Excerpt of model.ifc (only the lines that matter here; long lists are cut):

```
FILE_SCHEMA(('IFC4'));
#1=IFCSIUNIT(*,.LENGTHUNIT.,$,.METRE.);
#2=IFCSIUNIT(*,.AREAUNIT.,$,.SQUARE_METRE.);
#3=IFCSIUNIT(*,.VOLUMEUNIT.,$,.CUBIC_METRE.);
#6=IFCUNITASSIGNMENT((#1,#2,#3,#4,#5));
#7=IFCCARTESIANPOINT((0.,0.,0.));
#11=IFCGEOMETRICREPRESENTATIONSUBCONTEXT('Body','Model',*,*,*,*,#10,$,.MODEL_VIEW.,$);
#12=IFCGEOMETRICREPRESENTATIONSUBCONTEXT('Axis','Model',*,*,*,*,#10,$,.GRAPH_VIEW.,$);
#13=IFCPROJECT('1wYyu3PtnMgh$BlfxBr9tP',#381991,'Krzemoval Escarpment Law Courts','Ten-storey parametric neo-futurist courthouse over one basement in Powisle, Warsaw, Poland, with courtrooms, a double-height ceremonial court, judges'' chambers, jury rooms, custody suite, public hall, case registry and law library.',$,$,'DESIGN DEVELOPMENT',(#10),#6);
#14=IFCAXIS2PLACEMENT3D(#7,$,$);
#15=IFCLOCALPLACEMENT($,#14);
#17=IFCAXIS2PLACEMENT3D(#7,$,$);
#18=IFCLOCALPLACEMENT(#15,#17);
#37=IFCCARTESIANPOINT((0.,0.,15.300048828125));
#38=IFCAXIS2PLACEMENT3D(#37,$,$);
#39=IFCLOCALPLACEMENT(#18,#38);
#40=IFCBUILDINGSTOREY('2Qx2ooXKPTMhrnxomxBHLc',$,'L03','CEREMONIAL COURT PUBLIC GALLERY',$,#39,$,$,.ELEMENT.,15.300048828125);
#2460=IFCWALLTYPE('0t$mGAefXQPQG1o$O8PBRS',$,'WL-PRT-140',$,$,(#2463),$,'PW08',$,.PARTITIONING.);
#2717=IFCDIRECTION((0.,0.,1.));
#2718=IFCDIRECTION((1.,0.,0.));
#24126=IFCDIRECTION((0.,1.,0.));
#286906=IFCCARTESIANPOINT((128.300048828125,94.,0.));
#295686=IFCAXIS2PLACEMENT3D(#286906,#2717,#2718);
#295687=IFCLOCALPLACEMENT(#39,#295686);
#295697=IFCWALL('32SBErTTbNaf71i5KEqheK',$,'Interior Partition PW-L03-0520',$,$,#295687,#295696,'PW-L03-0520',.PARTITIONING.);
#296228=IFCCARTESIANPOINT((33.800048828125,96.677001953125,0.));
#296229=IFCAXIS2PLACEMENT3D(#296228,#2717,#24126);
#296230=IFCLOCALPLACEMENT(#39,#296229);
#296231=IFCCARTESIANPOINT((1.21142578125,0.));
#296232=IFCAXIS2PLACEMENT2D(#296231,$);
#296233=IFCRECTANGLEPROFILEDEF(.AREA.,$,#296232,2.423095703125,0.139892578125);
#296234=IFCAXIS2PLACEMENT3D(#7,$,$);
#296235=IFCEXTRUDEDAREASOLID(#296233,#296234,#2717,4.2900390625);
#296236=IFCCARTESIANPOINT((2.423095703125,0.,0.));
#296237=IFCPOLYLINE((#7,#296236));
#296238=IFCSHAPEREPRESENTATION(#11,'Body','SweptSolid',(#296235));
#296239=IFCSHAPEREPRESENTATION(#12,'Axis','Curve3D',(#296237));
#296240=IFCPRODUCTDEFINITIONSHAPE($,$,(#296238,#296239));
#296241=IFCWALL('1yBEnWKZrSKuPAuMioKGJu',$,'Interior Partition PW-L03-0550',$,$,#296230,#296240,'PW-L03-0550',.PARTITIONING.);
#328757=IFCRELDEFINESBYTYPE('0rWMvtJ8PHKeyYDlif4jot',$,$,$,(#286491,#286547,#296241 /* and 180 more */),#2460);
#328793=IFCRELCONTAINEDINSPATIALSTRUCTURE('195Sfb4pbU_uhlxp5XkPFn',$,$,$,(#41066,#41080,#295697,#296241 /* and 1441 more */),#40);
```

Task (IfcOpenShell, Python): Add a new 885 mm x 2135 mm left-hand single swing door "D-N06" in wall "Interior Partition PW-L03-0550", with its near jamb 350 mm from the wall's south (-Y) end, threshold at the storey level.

```python
import numpy as np
import ifcopenshell
import ifcopenshell.api.feature
import ifcopenshell.api.geometry
import ifcopenshell.api.root
import ifcopenshell.api.spatial
import ifcopenshell.geom
import ifcopenshell.util.element
import ifcopenshell.util.placement
import ifcopenshell.util.representation
import ifcopenshell.util.shape
import ifcopenshell.util.unit

model = ifcopenshell.open("model.ifc")
unit_scale = ifcopenshell.util.unit.calculate_unit_scale(model)
settings = ifcopenshell.geom.settings()


def volume(element):
    """Net volume in cubic metres, openings subtracted."""
    shape = ifcopenshell.geom.create_shape(settings, element)
    return ifcopenshell.util.shape.get_volume(shape.geometry)


wall = model.by_guid("1yBEnWKZrSKuPAuMioKGJu")
storey = ifcopenshell.util.element.get_container(wall, ifc_class="IfcBuildingStorey")
context = ifcopenshell.util.representation.get_context(model, "Model", "Body", "MODEL_VIEW")
before = volume(wall)

width, height, from_end, sill = 0.885, 2.135, 0.35, 0.0  # metres

# The wall runs along its own X axis, and the end named is its -X end.
wall_shape = ifcopenshell.geom.create_shape(settings, wall)
x, y, z = ifcopenshell.util.shape.get_vertices(wall_shape.geometry).T
start = x.min() + from_end
face, thickness = float(y.min()), float(y.max() - y.min())
wall_matrix = ifcopenshell.util.placement.get_local_placement(wall.ObjectPlacement)
level = ifcopenshell.util.placement.get_local_placement(storey.ObjectPlacement)[2, 3]


def in_wall(x, y):
    """Placement at x, y metres in the wall's axes, at sill height."""
    matrix = wall_matrix.copy()
    matrix[:, 3] = wall_matrix @ np.array([x / unit_scale, y / unit_scale, 0.0, 1.0])
    matrix[2, 3] = level + sill / unit_scale
    return matrix


# Opening: a box that overshoots both wall faces by 50 mm.
opening = ifcopenshell.api.root.create_entity(model, ifc_class="IfcOpeningElement", predefined_type="OPENING")
box = ifcopenshell.api.geometry.add_wall_representation(
    model, context=context, length=width, height=height, thickness=thickness + 0.1
)
ifcopenshell.api.geometry.assign_representation(model, product=opening, representation=box)
ifcopenshell.api.geometry.edit_object_placement(model, product=opening, matrix=in_wall(start, face - 0.05), is_si=False)
ifcopenshell.api.feature.add_feature(model, feature=opening, element=wall)

door = ifcopenshell.api.root.create_entity(model, ifc_class="IfcDoor", name="D-N06", predefined_type="DOOR")
door.OverallWidth, door.OverallHeight = width / unit_scale, height / unit_scale
door.OperationType = "SINGLE_SWING_LEFT"
body = ifcopenshell.api.geometry.add_door_representation(
    model,
    context=context,
    overall_width=door.OverallWidth,
    overall_height=door.OverallHeight,
    operation_type="SINGLE_SWING_LEFT",
    lining_properties={"LiningDepth": thickness / unit_scale, "ThresholdDepth": thickness / unit_scale},
)
ifcopenshell.api.geometry.assign_representation(model, product=door, representation=body)
ifcopenshell.api.spatial.assign_container(model, products=[door], relating_structure=storey)
ifcopenshell.api.feature.add_filling(model, opening=opening, element=door)

# The lining spans the wall, so the door starts at the wall face.
ifcopenshell.api.geometry.edit_object_placement(model, product=door, matrix=in_wall(start, face), is_si=False)

after = volume(wall)

print(f"wall volume {before:.3f} -> {after:.3f} m3")

model.write("model-out.ifc")
```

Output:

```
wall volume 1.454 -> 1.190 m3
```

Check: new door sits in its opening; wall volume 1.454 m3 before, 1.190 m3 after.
